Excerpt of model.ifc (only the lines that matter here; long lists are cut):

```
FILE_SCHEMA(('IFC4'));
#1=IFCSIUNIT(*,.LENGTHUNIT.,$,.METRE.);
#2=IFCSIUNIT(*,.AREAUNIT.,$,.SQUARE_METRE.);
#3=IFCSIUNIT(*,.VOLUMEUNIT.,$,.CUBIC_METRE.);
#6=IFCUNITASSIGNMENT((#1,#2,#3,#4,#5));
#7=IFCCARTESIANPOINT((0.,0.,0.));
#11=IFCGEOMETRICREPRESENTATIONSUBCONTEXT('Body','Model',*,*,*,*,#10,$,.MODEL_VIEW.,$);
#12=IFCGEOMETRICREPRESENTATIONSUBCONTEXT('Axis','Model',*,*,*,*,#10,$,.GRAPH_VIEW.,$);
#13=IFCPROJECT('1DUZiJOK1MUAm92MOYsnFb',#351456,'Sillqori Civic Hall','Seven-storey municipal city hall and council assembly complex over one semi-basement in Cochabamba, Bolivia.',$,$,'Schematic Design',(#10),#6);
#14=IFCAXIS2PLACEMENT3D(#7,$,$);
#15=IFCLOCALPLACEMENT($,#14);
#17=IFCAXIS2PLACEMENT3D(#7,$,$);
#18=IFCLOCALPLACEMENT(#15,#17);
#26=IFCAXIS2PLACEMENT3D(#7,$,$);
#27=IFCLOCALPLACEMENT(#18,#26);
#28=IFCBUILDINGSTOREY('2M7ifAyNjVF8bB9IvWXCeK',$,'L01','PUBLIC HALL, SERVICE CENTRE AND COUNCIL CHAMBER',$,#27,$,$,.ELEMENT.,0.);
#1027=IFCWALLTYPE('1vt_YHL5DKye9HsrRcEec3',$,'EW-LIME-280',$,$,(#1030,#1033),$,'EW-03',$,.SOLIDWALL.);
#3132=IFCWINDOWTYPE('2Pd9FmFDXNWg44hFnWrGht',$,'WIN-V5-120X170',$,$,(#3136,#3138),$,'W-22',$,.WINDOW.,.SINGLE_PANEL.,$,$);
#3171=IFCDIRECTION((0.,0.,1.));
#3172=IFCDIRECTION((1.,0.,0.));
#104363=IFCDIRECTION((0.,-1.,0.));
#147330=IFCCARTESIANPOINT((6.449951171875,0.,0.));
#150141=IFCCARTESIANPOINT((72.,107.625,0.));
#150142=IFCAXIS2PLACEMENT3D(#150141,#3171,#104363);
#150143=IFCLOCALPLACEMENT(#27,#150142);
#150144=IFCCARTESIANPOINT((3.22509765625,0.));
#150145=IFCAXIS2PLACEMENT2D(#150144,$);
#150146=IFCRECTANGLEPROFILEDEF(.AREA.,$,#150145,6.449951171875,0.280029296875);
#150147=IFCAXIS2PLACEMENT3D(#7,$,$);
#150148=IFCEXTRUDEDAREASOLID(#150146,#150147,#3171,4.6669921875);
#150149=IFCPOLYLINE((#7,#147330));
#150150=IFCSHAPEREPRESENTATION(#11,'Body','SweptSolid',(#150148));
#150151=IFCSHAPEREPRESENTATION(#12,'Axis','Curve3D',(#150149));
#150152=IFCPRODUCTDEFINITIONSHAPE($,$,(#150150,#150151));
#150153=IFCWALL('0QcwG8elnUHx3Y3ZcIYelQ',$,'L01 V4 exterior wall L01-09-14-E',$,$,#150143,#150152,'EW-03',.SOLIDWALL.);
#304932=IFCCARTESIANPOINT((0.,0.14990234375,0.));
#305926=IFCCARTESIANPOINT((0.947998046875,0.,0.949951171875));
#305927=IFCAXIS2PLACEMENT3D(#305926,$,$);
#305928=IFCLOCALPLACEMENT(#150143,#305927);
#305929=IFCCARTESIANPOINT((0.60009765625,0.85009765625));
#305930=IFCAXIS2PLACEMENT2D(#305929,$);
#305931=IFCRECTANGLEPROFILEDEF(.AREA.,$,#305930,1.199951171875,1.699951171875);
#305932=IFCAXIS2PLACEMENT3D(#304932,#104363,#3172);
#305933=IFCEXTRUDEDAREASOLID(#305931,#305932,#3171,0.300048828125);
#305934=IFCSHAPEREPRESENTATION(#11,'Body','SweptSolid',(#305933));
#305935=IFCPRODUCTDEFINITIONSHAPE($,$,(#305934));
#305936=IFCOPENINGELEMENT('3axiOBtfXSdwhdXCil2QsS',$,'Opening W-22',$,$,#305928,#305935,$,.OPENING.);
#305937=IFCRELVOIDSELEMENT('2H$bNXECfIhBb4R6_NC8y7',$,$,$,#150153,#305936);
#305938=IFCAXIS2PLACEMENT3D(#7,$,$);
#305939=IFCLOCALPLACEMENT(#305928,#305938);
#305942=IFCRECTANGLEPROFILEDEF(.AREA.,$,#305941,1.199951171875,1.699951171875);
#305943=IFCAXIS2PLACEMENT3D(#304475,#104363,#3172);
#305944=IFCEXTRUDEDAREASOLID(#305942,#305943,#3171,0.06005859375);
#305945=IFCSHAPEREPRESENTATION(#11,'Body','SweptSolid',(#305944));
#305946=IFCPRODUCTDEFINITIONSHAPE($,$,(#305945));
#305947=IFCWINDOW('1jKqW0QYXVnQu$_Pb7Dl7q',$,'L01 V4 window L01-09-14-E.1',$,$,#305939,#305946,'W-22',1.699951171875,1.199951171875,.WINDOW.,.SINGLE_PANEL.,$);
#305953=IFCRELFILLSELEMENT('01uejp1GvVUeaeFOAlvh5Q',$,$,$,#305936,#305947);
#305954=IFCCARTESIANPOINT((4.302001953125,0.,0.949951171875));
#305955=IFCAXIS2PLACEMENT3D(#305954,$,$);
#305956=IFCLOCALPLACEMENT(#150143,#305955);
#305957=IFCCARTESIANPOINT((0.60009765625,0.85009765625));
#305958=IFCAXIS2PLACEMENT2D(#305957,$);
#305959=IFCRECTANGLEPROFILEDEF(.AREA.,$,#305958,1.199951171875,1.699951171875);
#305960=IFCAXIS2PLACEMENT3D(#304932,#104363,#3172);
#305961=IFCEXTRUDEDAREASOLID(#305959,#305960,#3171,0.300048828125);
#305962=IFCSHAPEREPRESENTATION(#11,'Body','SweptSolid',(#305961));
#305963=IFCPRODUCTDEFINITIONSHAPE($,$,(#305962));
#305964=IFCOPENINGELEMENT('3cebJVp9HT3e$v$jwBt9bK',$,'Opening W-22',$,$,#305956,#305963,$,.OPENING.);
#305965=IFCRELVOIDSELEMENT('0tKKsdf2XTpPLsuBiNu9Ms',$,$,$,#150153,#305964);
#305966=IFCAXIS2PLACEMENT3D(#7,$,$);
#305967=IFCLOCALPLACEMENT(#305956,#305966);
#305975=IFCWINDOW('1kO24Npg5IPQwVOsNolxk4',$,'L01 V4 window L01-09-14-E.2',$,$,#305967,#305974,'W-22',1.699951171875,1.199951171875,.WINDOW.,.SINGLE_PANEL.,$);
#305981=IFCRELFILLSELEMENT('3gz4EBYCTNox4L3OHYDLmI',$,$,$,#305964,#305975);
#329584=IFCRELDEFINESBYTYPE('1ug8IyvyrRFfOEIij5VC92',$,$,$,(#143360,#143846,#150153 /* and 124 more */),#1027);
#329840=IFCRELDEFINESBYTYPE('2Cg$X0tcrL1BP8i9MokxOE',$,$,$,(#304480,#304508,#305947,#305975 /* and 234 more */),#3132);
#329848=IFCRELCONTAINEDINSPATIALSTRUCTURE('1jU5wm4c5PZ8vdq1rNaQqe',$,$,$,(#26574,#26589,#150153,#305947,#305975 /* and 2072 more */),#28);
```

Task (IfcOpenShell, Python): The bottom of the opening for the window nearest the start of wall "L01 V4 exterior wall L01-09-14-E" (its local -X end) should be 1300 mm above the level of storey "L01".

```python
import numpy as np
import ifcopenshell
import ifcopenshell.api.geometry
import ifcopenshell.geom
import ifcopenshell.util.element
import ifcopenshell.util.placement
import ifcopenshell.util.shape
import ifcopenshell.util.unit

model = ifcopenshell.open("model.ifc")
unit_scale = ifcopenshell.util.unit.calculate_unit_scale(model)

window = model.by_id(305947)
opening = window.FillsVoids[0].RelatingOpeningElement
storey = ifcopenshell.util.element.get_container(window, ifc_class="IfcBuildingStorey")
level = ifcopenshell.util.placement.get_local_placement(storey.ObjectPlacement)[2, 3]

# The opening's origin need not be at the sill, so measure its lowest point.
shape = ifcopenshell.geom.create_shape(ifcopenshell.geom.settings(), opening)
bottom = ifcopenshell.util.shape.get_shape_bottom_elevation(shape, shape.geometry) / unit_scale
dz = level + 1.3 / unit_scale - bottom

shift = np.array([0.0, 0.0, dz])
# The window is placed relative to its opening, so it follows when the opening moves.
matrix = ifcopenshell.util.placement.get_local_placement(opening.ObjectPlacement)
matrix[:3, 3] += shift
ifcopenshell.api.geometry.edit_object_placement(
    model, product=opening, matrix=matrix, is_si=False, should_transform_children=True
)

print(f"moved by {dz * unit_scale:+.3f} m")

model.write("model_edited.ifc")
```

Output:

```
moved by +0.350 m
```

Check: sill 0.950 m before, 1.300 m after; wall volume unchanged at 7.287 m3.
